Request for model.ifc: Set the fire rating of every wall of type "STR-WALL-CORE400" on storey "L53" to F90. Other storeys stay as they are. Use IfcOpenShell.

First a look at what the model holds.

```python
import ifcopenshell
import ifcopenshell.util.element

model = ifcopenshell.open("model.ifc")
print(model.schema)
storey = next(s for s in model.by_type("IfcBuildingStorey") if s.Name == "L53")
walls = [e for e in ifcopenshell.util.element.get_decomposition(storey) if e.is_a("IfcWall")]
seen = {}
for e in walls:
    element_type = ifcopenshell.util.element.get_type(e)
    key = (element_type.Name if element_type != e and element_type else None, ifcopenshell.util.element.get_pset(e, "Pset_WallCommon", "FireRating"))
    seen[key] = seen.get(key, 0) + 1
for (name, value), count in sorted(seen.items(), key=str):
    print(count, "x", name, "|", value)
```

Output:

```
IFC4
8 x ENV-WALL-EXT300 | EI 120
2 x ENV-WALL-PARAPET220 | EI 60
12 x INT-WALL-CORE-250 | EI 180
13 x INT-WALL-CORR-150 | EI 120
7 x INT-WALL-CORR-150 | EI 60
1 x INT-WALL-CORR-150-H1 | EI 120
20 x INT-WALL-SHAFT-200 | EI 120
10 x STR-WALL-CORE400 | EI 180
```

```python
import ifcopenshell
import ifcopenshell.api.pset
import ifcopenshell.util.element

model = ifcopenshell.open("model.ifc")

storey = next(s for s in model.by_type("IfcBuildingStorey") if s.Name == "L53")
walls = [e for e in ifcopenshell.util.element.get_decomposition(storey) if e.is_a("IfcWall")]

count = 0
for e in walls:
    element_type = ifcopenshell.util.element.get_type(e)
    if element_type in (None, e) or element_type.Name != "STR-WALL-CORE400":
        continue
    found = ifcopenshell.util.element.get_pset(e, "Pset_WallCommon", should_inherit=False)
    if found:
        pset = model.by_id(found["id"])
        if len(ifcopenshell.util.element.get_elements_by_pset(pset)) > 1:
            pset = ifcopenshell.api.pset.unshare_pset(model, products=[e], pset=pset)[0]
    else:
        pset = ifcopenshell.api.pset.add_pset(model, product=e, name="Pset_WallCommon")
    ifcopenshell.api.pset.edit_pset(model, pset=pset, properties={"FireRating": "F90"})
    count += 1

print(count, "walls updated")

model.write("model_v2.ifc")
```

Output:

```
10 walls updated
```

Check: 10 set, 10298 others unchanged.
